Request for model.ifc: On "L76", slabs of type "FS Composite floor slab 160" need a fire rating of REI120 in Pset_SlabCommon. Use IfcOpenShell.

First a look at what the model holds.

```python
import ifcopenshell
import ifcopenshell.util.element

model = ifcopenshell.open("model.ifc")
print(model.schema)
storey = next(s for s in model.by_type("IfcBuildingStorey") if s.Name == "L76")
slabs = [e for e in ifcopenshell.util.element.get_decomposition(storey) if e.is_a("IfcSlab")]
seen = {}
for e in slabs:
    element_type = ifcopenshell.util.element.get_type(e)
    key = (element_type.Name if element_type != e and element_type else None, ifcopenshell.util.element.get_pset(e, "Pset_SlabCommon", "FireRating"))
    seen[key] = seen.get(key, 0) + 1
for (name, value), count in sorted(seen.items(), key=str):
    print(count, "x", name, "|", value)
```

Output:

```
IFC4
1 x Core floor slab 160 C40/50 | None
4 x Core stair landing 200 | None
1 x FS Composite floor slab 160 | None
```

```python
import ifcopenshell
import ifcopenshell.api.pset
import ifcopenshell.util.element

model = ifcopenshell.open("model.ifc")

storey = next(s for s in model.by_type("IfcBuildingStorey") if s.Name == "L76")
slabs = [e for e in ifcopenshell.util.element.get_decomposition(storey) if e.is_a("IfcSlab")]

count = 0
for e in slabs:
    element_type = ifcopenshell.util.element.get_type(e)
    if element_type in (None, e) or element_type.Name != "FS Composite floor slab 160":
        continue
    found = ifcopenshell.util.element.get_pset(e, "Pset_SlabCommon", should_inherit=False)
    if found:
        pset = model.by_id(found["id"])
        if len(ifcopenshell.util.element.get_elements_by_pset(pset)) > 1:
            pset = ifcopenshell.api.pset.unshare_pset(model, products=[e], pset=pset)[0]
    else:
        pset = ifcopenshell.api.pset.add_pset(model, product=e, name="Pset_SlabCommon")
    ifcopenshell.api.pset.edit_pset(model, pset=pset, properties={"FireRating": "REI120"})
    count += 1

print(count, "slabs updated")

model.write("model-out.ifc")
```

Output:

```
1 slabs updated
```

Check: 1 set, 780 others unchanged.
